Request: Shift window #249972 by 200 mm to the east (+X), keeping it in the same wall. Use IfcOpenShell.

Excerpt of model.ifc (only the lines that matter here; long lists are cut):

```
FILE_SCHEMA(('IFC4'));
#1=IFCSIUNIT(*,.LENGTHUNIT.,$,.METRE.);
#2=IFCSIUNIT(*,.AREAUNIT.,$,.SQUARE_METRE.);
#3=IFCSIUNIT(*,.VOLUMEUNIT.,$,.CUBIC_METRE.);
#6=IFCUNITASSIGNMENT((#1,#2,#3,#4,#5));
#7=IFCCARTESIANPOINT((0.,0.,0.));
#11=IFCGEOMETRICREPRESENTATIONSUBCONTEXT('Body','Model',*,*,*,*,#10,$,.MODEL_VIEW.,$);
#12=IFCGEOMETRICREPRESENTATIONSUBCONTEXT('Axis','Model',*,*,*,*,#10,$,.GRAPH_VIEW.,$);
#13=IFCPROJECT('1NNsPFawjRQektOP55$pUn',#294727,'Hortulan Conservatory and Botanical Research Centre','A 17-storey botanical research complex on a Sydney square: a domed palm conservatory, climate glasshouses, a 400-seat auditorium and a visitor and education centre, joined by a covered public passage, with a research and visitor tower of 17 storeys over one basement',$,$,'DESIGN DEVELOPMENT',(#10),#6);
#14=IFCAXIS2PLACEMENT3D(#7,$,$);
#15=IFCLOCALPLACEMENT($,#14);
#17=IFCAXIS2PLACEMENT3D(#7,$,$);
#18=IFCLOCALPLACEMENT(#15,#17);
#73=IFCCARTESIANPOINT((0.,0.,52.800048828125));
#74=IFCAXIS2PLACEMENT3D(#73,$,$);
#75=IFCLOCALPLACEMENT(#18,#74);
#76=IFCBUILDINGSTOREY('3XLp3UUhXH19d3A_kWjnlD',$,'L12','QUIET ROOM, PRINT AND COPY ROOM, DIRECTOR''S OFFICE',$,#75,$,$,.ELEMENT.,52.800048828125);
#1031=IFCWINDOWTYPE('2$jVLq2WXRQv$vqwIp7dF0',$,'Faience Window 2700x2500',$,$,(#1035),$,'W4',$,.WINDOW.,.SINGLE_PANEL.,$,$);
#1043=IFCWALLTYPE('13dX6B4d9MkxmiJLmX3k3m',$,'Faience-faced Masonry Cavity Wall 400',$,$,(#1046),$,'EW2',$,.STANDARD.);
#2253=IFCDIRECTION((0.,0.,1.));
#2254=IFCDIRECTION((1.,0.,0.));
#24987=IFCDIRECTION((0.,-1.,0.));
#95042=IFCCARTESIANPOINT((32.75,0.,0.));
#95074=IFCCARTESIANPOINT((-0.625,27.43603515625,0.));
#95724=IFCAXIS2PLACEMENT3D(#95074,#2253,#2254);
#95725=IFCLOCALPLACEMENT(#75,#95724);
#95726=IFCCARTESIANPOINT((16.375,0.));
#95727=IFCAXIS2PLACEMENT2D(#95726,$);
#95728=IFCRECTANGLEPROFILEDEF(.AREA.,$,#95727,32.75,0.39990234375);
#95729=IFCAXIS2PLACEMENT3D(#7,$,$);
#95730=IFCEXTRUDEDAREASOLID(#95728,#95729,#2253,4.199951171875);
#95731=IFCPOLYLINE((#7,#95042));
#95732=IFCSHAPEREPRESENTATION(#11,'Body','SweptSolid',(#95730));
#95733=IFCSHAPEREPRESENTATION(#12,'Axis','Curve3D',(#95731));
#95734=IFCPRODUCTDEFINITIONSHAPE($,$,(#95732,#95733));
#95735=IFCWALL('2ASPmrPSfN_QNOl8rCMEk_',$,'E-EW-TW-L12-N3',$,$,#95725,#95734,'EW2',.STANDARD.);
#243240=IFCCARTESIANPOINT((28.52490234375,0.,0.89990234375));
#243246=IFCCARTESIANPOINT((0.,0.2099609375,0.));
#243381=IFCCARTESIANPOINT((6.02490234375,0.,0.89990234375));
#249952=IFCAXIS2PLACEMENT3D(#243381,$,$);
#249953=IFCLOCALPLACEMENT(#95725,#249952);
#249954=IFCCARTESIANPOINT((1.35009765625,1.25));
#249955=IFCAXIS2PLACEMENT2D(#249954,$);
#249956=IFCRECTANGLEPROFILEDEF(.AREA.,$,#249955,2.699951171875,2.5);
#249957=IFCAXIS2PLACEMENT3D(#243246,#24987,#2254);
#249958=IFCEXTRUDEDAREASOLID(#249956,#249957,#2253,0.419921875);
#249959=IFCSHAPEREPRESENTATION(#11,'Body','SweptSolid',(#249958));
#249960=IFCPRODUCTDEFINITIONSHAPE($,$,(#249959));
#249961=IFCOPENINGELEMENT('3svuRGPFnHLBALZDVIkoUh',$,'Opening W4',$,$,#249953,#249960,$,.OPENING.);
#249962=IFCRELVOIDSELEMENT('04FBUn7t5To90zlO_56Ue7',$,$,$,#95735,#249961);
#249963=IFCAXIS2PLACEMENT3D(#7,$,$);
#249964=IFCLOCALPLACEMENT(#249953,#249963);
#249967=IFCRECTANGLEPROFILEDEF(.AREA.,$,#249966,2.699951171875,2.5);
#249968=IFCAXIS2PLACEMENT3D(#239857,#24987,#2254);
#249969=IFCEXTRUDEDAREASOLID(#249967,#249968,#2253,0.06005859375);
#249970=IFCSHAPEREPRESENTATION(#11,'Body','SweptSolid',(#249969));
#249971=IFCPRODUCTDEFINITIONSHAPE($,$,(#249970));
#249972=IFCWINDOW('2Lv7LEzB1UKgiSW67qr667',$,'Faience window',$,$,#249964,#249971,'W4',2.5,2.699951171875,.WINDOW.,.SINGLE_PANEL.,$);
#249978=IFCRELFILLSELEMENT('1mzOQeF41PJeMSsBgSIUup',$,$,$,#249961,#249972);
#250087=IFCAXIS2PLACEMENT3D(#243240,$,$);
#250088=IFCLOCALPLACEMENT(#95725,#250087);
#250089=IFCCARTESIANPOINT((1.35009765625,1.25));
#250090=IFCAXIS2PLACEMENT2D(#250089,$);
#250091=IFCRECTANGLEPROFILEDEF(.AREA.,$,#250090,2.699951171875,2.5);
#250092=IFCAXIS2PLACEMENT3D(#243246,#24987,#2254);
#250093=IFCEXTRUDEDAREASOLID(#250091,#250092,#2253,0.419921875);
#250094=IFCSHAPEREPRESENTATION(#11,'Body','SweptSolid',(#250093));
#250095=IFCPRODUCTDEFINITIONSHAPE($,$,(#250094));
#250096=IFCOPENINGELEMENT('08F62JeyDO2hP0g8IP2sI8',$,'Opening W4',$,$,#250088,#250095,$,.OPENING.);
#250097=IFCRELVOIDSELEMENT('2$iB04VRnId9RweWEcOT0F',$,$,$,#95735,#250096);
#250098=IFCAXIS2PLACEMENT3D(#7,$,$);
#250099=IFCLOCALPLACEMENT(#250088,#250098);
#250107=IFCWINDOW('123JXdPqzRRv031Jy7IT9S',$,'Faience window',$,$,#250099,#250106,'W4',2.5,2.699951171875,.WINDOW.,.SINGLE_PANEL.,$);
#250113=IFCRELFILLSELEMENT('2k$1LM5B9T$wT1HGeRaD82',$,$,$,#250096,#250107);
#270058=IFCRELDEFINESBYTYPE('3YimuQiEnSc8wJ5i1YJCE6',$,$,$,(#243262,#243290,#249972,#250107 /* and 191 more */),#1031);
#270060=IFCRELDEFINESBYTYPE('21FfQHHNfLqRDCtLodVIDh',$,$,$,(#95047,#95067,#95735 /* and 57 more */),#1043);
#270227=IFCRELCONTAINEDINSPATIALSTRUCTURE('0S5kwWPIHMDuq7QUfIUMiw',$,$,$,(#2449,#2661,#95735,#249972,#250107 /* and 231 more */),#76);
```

```python
import ifcopenshell
import ifcopenshell.api.geometry
import ifcopenshell.util.placement

model = ifcopenshell.open("model.ifc")

window = model.by_guid("2Lv7LEzB1UKgiSW67qr667")
opening = window.FillsVoids[0].RelatingOpeningElement
wall = opening.VoidsElements[0].RelatingBuildingElement

wall_matrix = ifcopenshell.util.placement.get_local_placement(wall.ObjectPlacement)
shift = wall_matrix[:3, 0] * 0.2
before = ifcopenshell.util.placement.get_local_placement(window.ObjectPlacement)[:3, 3].copy()

# The window is placed relative to its opening, so it follows when the opening moves.
matrix = ifcopenshell.util.placement.get_local_placement(opening.ObjectPlacement)
matrix[:3, 3] += shift
ifcopenshell.api.geometry.edit_object_placement(
    model, product=opening, matrix=matrix, is_si=False, should_transform_children=True
)

after = ifcopenshell.util.placement.get_local_placement(window.ObjectPlacement)[:3, 3]
print("window moved by", (after - before).round(3) + 0.0)

model.write("model_edited.ifc")
```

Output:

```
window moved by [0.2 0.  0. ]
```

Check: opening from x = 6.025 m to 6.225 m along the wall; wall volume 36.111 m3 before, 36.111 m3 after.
